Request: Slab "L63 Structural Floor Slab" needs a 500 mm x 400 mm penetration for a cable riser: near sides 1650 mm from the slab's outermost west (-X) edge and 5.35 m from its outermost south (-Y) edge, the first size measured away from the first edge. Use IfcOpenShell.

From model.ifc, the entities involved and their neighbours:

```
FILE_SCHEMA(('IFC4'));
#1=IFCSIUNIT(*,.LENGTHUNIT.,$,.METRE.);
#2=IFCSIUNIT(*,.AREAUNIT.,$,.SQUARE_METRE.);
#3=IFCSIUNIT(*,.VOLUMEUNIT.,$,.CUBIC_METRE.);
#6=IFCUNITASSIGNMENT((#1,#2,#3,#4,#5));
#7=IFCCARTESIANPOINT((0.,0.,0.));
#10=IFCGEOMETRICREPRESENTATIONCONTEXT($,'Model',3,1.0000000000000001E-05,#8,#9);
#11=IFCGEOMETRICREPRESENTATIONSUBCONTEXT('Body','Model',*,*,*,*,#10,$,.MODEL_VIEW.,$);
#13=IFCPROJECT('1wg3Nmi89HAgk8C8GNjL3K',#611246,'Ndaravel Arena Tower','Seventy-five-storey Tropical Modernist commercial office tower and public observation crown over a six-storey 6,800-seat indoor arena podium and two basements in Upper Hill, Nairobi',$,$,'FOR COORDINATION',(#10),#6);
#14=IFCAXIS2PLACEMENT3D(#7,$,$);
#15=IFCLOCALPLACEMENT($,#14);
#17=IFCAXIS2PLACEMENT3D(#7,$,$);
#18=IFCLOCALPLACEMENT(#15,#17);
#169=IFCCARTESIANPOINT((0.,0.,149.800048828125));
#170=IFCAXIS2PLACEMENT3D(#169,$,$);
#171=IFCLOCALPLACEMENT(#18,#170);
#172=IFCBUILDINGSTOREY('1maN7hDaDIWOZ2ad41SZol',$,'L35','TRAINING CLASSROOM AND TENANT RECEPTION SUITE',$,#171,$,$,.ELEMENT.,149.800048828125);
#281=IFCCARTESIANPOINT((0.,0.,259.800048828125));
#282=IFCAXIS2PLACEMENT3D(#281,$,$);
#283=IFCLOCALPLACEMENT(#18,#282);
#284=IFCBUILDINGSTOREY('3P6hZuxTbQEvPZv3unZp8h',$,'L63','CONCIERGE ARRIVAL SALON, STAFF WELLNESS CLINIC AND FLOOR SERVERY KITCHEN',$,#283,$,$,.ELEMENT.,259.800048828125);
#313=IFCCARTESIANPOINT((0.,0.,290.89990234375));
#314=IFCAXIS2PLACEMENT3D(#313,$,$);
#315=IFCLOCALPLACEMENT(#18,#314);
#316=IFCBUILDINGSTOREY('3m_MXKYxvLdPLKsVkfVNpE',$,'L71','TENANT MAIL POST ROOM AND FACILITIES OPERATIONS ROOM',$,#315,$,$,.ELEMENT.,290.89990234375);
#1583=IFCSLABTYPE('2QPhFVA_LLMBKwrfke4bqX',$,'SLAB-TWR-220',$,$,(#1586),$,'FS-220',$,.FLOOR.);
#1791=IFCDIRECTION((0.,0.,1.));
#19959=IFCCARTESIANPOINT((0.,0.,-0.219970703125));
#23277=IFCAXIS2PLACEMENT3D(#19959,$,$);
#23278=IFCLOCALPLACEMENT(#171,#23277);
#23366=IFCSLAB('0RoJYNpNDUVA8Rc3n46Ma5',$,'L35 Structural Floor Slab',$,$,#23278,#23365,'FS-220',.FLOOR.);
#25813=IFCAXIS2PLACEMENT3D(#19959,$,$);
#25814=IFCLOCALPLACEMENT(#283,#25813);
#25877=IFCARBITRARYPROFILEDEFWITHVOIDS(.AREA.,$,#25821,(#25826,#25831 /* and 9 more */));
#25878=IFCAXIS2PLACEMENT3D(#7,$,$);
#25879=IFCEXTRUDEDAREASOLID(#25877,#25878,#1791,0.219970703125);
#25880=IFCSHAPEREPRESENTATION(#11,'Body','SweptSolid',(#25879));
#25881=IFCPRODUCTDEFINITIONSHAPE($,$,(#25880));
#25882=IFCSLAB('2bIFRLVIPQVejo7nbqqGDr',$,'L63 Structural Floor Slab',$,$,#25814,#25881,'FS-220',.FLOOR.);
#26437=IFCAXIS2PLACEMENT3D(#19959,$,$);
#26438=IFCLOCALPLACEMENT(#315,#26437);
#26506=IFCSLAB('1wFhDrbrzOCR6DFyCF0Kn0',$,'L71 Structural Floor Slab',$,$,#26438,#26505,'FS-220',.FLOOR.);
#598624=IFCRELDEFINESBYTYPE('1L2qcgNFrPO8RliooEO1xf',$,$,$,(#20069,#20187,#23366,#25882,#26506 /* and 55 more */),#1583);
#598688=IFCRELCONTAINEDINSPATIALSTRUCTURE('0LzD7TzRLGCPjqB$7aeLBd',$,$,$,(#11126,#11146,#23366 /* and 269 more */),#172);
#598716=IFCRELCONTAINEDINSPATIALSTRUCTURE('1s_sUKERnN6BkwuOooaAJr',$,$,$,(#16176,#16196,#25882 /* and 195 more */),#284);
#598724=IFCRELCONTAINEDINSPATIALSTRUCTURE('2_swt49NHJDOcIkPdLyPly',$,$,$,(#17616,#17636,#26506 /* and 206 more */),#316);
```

```python
import numpy as np
import ifcopenshell
import ifcopenshell.api.feature
import ifcopenshell.api.geometry
import ifcopenshell.api.root
import ifcopenshell.geom
import ifcopenshell.util.placement
import ifcopenshell.util.representation
import ifcopenshell.util.shape
import ifcopenshell.util.unit

model = ifcopenshell.open("model.ifc")
unit_scale = ifcopenshell.util.unit.calculate_unit_scale(model)
settings = ifcopenshell.geom.settings()


def volume(element):
    """Net volume in cubic metres, openings subtracted."""
    shape = ifcopenshell.geom.create_shape(settings, element)
    return ifcopenshell.util.shape.get_volume(shape.geometry)


slab = model.by_guid("2bIFRLVIPQVejo7nbqqGDr")
before = volume(slab)

# Extent in the slab's own axes, in metres. The edges named are its -X and -Y sides.
slab_shape = ifcopenshell.geom.create_shape(settings, slab)
vertices = ifcopenshell.util.shape.get_vertices(slab_shape.geometry)
x_min, y_min, bottom = vertices.min(axis=0)
top = vertices[:, 2].max()

opening = ifcopenshell.api.root.create_entity(model, ifc_class="IfcOpeningElement", name="Cable riser opening", predefined_type="OPENING")
context = ifcopenshell.util.representation.get_context(model, "Model", "Body", "MODEL_VIEW")
width, depth = 0.5, 0.4
outline = [(0.0, 0.0), (width, 0.0), (width, depth), (0.0, depth), (0.0, 0.0)]
# Overshoot both faces by 50 mm so the cut is clean.
shape = ifcopenshell.api.geometry.add_slab_representation(
    model, context=context, depth=top - bottom + 0.1, polyline=outline
)
ifcopenshell.api.geometry.assign_representation(model, product=opening, representation=shape)

matrix = ifcopenshell.util.placement.get_local_placement(slab.ObjectPlacement)
matrix[:, 3] = matrix @ np.append(np.array([x_min + 1.65, y_min + 5.35, bottom - 0.05]) / unit_scale, 1.0)
ifcopenshell.api.geometry.edit_object_placement(model, product=opening, matrix=matrix, is_si=False)
ifcopenshell.api.feature.add_feature(model, feature=opening, element=slab)

after = volume(slab)

print(f"slab volume {before:.3f} -> {after:.3f} m3")

model.write("model_edited.ifc")
```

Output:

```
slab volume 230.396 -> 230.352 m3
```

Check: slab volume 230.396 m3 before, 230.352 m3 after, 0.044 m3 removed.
